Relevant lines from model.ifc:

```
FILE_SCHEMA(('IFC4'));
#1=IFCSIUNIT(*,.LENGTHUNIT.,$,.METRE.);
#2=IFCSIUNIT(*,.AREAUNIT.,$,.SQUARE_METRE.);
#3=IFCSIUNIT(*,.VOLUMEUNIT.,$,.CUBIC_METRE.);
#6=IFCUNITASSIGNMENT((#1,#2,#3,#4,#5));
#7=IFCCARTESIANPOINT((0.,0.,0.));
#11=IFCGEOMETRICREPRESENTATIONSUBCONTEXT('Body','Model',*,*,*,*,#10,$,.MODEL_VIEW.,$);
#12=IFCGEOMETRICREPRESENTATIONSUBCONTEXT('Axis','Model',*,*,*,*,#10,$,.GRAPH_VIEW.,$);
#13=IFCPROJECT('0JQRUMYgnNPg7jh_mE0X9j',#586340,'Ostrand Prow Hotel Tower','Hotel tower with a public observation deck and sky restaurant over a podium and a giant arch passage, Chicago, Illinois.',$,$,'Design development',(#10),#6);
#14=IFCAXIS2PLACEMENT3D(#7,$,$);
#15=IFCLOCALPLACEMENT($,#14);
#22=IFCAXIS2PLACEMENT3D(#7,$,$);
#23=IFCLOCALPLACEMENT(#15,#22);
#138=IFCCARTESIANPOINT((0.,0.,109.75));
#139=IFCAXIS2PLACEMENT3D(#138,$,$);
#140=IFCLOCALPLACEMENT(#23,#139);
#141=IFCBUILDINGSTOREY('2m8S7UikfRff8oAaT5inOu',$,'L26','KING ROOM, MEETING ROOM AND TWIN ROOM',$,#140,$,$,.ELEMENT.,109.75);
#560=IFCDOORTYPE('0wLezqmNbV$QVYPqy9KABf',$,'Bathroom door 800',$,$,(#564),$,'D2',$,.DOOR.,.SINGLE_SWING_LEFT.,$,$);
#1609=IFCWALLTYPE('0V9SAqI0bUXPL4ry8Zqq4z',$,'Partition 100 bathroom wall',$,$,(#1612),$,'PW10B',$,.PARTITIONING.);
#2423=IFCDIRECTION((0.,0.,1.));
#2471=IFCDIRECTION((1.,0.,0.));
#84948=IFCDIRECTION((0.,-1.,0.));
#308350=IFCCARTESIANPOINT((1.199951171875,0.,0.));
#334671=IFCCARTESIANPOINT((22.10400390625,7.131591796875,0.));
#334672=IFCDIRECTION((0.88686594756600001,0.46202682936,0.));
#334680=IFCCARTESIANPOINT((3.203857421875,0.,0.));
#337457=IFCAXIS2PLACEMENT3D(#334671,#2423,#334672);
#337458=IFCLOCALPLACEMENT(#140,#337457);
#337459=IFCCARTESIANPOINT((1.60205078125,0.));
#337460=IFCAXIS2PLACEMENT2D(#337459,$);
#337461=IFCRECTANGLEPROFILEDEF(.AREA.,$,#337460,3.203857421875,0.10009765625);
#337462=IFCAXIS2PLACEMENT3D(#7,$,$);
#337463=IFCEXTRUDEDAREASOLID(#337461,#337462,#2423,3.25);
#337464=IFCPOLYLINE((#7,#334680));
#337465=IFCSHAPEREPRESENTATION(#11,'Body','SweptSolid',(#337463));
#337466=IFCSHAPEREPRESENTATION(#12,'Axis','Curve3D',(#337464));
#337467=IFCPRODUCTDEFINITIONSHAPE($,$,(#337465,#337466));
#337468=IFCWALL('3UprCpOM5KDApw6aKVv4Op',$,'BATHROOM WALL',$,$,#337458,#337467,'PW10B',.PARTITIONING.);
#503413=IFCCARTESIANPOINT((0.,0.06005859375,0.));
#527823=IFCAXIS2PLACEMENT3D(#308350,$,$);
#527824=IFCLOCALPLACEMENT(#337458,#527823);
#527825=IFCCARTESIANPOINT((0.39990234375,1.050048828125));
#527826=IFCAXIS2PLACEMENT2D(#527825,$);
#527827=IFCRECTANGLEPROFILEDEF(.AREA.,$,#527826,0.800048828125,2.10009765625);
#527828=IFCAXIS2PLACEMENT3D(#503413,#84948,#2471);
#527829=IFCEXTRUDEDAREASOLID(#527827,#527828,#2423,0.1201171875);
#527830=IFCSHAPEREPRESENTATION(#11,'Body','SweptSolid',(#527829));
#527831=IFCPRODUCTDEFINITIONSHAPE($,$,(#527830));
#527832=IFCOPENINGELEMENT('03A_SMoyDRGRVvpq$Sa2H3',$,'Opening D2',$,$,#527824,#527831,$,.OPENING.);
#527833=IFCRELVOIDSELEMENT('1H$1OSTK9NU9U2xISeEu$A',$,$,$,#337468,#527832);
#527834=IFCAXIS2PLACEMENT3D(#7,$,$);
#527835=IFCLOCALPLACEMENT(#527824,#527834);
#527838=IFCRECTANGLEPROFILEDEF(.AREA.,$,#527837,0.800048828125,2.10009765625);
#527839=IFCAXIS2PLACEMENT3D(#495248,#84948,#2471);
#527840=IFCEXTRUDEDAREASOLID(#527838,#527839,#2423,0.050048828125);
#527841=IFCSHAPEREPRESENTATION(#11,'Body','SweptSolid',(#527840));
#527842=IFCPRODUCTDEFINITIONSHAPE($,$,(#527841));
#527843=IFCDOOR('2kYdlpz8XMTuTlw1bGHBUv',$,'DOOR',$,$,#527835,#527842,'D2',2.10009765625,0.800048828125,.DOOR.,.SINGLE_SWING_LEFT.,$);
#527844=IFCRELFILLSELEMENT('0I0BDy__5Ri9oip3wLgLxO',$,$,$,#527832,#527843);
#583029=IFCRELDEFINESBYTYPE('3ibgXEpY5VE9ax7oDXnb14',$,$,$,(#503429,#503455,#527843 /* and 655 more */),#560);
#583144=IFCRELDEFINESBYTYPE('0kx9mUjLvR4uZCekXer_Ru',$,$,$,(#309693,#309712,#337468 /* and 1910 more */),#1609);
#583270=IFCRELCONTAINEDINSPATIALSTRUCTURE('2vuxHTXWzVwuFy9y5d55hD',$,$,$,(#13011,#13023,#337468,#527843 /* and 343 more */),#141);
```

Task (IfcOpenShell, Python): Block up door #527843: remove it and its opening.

```python
import ifcopenshell
import ifcopenshell.api.feature
import ifcopenshell.api.root
import ifcopenshell.geom
import ifcopenshell.util.shape

model = ifcopenshell.open("model.ifc")
settings = ifcopenshell.geom.settings()


def volume(element):
    """Net volume in cubic metres, openings subtracted."""
    shape = ifcopenshell.geom.create_shape(settings, element)
    return ifcopenshell.util.shape.get_volume(shape.geometry)


door = model.by_guid("2kYdlpz8XMTuTlw1bGHBUv")
opening = door.FillsVoids[0].RelatingOpeningElement
wall = opening.VoidsElements[0].RelatingBuildingElement
before = volume(wall)

ifcopenshell.api.root.remove_product(model, product=door)
ifcopenshell.api.feature.remove_feature(model, feature=opening)

after = volume(wall)

print(f"wall volume {before:.3f} -> {after:.3f} m3")

model.write("model_updated.ifc")
```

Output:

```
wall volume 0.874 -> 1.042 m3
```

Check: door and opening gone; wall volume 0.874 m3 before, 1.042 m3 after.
